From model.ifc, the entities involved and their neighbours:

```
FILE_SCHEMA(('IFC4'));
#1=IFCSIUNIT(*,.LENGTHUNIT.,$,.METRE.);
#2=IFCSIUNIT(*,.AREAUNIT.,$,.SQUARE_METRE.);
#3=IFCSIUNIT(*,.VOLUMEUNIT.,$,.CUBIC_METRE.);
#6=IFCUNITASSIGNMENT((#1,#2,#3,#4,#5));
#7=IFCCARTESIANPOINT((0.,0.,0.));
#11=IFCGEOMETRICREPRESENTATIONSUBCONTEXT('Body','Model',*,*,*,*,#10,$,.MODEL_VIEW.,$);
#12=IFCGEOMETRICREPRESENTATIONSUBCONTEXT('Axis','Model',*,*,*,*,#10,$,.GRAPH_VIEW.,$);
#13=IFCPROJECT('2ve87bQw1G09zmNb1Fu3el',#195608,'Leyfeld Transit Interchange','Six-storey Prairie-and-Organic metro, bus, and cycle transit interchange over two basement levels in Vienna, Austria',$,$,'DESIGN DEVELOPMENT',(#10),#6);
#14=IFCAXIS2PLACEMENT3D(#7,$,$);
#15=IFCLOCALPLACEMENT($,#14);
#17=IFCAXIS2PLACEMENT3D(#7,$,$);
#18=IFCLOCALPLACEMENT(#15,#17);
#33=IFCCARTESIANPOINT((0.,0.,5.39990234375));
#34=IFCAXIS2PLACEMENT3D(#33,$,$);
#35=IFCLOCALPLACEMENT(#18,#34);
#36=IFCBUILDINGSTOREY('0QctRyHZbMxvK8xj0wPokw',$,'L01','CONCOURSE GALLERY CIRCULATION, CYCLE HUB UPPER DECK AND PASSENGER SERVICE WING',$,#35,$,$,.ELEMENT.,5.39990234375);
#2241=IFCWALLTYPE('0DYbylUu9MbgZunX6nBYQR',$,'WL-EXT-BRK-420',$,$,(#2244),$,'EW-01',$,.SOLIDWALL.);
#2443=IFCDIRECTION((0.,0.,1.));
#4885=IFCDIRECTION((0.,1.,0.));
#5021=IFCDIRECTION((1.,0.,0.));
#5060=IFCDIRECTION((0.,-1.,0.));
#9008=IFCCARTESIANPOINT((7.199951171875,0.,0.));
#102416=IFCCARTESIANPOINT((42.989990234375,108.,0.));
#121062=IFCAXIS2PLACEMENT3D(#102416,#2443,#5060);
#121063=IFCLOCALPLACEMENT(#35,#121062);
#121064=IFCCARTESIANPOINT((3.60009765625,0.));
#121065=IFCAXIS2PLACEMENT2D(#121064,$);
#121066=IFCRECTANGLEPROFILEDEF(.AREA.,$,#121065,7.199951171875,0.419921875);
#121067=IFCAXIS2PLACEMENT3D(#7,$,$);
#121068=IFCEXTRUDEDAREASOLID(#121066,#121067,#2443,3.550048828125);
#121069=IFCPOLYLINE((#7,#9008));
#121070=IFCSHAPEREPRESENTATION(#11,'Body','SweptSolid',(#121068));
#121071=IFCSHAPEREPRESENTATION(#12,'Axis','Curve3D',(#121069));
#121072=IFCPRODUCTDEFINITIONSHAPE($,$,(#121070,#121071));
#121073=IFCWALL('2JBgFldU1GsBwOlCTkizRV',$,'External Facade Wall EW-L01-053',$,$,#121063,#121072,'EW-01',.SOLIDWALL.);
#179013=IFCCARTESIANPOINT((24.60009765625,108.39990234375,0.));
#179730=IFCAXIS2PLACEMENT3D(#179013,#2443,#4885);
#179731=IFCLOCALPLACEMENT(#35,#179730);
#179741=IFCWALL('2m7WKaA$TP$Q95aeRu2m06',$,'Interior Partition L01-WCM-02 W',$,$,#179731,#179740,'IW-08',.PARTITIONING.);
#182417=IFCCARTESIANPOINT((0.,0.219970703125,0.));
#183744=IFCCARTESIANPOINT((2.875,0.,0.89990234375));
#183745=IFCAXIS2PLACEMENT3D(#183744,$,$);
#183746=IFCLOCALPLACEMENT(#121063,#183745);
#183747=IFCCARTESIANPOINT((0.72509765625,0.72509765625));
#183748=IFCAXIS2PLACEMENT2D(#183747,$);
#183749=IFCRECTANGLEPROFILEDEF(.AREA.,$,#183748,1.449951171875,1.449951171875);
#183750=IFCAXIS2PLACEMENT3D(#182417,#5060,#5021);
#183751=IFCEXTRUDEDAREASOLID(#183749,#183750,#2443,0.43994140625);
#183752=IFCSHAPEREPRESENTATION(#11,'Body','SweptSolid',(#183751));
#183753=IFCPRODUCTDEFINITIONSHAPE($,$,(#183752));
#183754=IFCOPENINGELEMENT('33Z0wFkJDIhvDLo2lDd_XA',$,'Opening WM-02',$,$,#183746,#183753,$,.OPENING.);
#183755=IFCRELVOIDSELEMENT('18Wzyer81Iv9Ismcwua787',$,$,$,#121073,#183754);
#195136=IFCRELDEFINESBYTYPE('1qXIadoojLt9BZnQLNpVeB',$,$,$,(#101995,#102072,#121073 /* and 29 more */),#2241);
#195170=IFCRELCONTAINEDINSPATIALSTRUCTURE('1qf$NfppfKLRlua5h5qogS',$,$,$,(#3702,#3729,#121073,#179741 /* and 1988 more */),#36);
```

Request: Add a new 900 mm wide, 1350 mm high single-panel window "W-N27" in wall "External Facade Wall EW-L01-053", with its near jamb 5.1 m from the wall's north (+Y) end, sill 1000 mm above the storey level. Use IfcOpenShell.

```python
import numpy as np
import ifcopenshell
import ifcopenshell.api.feature
import ifcopenshell.api.geometry
import ifcopenshell.api.root
import ifcopenshell.api.spatial
import ifcopenshell.geom
import ifcopenshell.util.element
import ifcopenshell.util.placement
import ifcopenshell.util.representation
import ifcopenshell.util.shape
import ifcopenshell.util.unit

model = ifcopenshell.open("model.ifc")
unit_scale = ifcopenshell.util.unit.calculate_unit_scale(model)
settings = ifcopenshell.geom.settings()


def volume(element):
    """Net volume in cubic metres, openings subtracted."""
    shape = ifcopenshell.geom.create_shape(settings, element)
    return ifcopenshell.util.shape.get_volume(shape.geometry)


wall = model.by_id(121073)
storey = ifcopenshell.util.element.get_container(wall, ifc_class="IfcBuildingStorey")
context = ifcopenshell.util.representation.get_context(model, "Model", "Body", "MODEL_VIEW")
before = volume(wall)

width, height, from_end, sill = 0.9, 1.35, 5.1, 1  # metres

# The wall runs along its own X axis, and the end named is its -X end.
wall_shape = ifcopenshell.geom.create_shape(settings, wall)
x, y, z = ifcopenshell.util.shape.get_vertices(wall_shape.geometry).T
start = x.min() + from_end
face, thickness = float(y.min()), float(y.max() - y.min())
wall_matrix = ifcopenshell.util.placement.get_local_placement(wall.ObjectPlacement)
level = ifcopenshell.util.placement.get_local_placement(storey.ObjectPlacement)[2, 3]


def in_wall(x, y):
    """Placement at x, y metres in the wall's axes, at sill height."""
    matrix = wall_matrix.copy()
    matrix[:, 3] = wall_matrix @ np.array([x / unit_scale, y / unit_scale, 0.0, 1.0])
    matrix[2, 3] = level + sill / unit_scale
    return matrix


# Opening: a box that overshoots both wall faces by 50 mm.
opening = ifcopenshell.api.root.create_entity(model, ifc_class="IfcOpeningElement", predefined_type="OPENING")
box = ifcopenshell.api.geometry.add_wall_representation(
    model, context=context, length=width, height=height, thickness=thickness + 0.1
)
ifcopenshell.api.geometry.assign_representation(model, product=opening, representation=box)
ifcopenshell.api.geometry.edit_object_placement(model, product=opening, matrix=in_wall(start, face - 0.05), is_si=False)
ifcopenshell.api.feature.add_feature(model, feature=opening, element=wall)

window = ifcopenshell.api.root.create_entity(model, ifc_class="IfcWindow", name="W-N27", predefined_type="WINDOW")
window.OverallWidth, window.OverallHeight = width / unit_scale, height / unit_scale
window.PartitioningType = "SINGLE_PANEL"
body = ifcopenshell.api.geometry.add_window_representation(
    model,
    context=context,
    overall_width=window.OverallWidth,
    overall_height=window.OverallHeight,
    partition_type="SINGLE_PANEL",
)
ifcopenshell.api.geometry.assign_representation(model, product=window, representation=body)
ifcopenshell.api.spatial.assign_container(model, products=[window], relating_structure=storey)
ifcopenshell.api.feature.add_filling(model, opening=opening, element=window)

# Centre the window in the wall's thickness.
ifcopenshell.api.geometry.edit_object_placement(model, product=window, matrix=in_wall(start, face), is_si=False)
window_shape = ifcopenshell.geom.create_shape(settings, window)
depth = ifcopenshell.util.shape.get_vertices(window_shape.geometry)[:, 1]
offset = face + thickness / 2 - (depth.min() + depth.max()) / 2
ifcopenshell.api.geometry.edit_object_placement(model, product=window, matrix=in_wall(start, offset), is_si=False)

after = volume(wall)

print(f"wall volume {before:.3f} -> {after:.3f} m3")

model.write("model_edited.ifc")
```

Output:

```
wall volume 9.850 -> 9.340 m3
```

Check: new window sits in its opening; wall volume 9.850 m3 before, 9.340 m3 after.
